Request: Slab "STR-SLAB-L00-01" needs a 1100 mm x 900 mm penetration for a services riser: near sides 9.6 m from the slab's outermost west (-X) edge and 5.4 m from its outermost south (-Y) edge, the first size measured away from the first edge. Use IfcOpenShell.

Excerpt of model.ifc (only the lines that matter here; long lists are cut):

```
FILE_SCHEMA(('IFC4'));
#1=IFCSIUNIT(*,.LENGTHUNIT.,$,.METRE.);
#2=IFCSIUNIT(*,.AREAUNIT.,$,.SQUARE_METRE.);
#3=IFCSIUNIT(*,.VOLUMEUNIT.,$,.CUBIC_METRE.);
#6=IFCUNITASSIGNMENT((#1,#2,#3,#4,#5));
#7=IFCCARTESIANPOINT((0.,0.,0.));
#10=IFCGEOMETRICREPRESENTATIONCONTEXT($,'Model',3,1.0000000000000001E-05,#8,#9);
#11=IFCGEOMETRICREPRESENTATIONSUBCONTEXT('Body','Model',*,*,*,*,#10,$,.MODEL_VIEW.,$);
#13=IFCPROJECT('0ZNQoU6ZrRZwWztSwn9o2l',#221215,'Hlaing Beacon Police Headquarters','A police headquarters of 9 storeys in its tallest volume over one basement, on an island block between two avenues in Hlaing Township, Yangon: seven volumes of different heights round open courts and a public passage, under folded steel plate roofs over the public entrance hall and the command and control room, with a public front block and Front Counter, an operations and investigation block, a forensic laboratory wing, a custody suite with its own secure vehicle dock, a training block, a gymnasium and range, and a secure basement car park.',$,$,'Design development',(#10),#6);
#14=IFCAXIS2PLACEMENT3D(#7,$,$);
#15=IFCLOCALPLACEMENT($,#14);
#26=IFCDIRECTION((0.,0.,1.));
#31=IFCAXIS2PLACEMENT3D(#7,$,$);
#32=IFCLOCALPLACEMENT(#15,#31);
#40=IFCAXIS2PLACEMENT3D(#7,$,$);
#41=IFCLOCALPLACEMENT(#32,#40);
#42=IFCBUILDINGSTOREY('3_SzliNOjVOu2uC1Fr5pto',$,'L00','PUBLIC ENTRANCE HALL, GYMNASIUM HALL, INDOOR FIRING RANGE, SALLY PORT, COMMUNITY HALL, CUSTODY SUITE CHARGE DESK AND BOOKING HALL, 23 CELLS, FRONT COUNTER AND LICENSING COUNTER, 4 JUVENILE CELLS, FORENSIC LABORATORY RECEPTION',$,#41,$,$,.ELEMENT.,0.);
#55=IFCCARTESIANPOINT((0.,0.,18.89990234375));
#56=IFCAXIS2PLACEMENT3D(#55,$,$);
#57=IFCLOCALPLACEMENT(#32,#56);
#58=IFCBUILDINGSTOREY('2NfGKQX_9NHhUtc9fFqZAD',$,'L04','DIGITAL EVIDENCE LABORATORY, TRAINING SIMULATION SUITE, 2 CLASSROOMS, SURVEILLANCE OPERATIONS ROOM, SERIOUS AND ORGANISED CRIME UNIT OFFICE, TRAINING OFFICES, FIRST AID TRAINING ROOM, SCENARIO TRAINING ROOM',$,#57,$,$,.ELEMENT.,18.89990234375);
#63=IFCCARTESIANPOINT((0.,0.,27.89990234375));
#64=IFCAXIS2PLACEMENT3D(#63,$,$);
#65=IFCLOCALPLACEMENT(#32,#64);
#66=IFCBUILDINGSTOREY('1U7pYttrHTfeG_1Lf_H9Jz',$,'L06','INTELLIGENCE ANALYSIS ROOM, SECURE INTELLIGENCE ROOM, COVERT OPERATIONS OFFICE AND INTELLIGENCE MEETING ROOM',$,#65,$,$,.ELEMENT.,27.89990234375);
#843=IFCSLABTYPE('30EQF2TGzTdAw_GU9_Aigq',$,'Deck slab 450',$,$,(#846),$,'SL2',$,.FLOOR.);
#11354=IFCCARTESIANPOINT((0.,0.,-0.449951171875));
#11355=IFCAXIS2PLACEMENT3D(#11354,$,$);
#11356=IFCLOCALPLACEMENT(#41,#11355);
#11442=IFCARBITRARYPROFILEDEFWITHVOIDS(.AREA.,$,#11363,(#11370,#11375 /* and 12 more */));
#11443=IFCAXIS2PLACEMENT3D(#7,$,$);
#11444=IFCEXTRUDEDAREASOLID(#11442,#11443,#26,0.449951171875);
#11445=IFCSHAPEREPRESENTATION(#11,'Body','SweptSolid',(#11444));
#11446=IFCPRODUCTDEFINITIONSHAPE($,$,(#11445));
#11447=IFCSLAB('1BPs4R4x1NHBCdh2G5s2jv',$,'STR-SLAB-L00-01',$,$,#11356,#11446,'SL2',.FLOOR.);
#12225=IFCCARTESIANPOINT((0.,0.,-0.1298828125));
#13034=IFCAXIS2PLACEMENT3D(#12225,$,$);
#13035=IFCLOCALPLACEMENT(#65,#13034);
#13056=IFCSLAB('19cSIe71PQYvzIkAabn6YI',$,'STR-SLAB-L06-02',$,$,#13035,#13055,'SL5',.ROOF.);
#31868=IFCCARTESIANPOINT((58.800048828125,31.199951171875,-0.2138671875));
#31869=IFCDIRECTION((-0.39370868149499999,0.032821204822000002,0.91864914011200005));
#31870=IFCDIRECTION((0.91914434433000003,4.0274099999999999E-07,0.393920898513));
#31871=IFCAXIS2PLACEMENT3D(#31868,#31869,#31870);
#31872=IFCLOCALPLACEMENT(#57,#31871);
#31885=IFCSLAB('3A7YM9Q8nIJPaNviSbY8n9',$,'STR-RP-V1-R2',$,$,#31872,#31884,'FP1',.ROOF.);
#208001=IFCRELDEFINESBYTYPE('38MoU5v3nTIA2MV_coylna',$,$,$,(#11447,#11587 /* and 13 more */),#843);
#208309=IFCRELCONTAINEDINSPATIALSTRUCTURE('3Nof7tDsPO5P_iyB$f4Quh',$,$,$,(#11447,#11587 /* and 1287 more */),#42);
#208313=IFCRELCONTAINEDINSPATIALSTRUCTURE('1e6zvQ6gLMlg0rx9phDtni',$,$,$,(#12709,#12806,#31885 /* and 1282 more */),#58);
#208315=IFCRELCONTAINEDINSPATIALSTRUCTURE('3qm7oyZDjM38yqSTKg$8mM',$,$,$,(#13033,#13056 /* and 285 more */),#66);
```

```python
import numpy as np
import ifcopenshell
import ifcopenshell.api.feature
import ifcopenshell.api.geometry
import ifcopenshell.api.root
import ifcopenshell.geom
import ifcopenshell.util.placement
import ifcopenshell.util.representation
import ifcopenshell.util.shape
import ifcopenshell.util.unit

model = ifcopenshell.open("model.ifc")
unit_scale = ifcopenshell.util.unit.calculate_unit_scale(model)
settings = ifcopenshell.geom.settings()


def volume(element):
    """Net volume in cubic metres, openings subtracted."""
    shape = ifcopenshell.geom.create_shape(settings, element)
    return ifcopenshell.util.shape.get_volume(shape.geometry)


slab = model.by_guid("1BPs4R4x1NHBCdh2G5s2jv")
before = volume(slab)

# Extent in the slab's own axes, in metres. The edges named are its -X and -Y sides.
slab_shape = ifcopenshell.geom.create_shape(settings, slab)
vertices = ifcopenshell.util.shape.get_vertices(slab_shape.geometry)
x_min, y_min, bottom = vertices.min(axis=0)
top = vertices[:, 2].max()

opening = ifcopenshell.api.root.create_entity(model, ifc_class="IfcOpeningElement", name="Services riser opening", predefined_type="OPENING")
context = ifcopenshell.util.representation.get_context(model, "Model", "Body", "MODEL_VIEW")
width, depth = 1.1, 0.9
outline = [(0.0, 0.0), (width, 0.0), (width, depth), (0.0, depth), (0.0, 0.0)]
# Overshoot both faces by 50 mm so the cut is clean.
shape = ifcopenshell.api.geometry.add_slab_representation(
    model, context=context, depth=top - bottom + 0.1, polyline=outline
)
ifcopenshell.api.geometry.assign_representation(model, product=opening, representation=shape)

matrix = ifcopenshell.util.placement.get_local_placement(slab.ObjectPlacement)
matrix[:, 3] = matrix @ np.append(np.array([x_min + 9.6, y_min + 5.4, bottom - 0.05]) / unit_scale, 1.0)
ifcopenshell.api.geometry.edit_object_placement(model, product=opening, matrix=matrix, is_si=False)
ifcopenshell.api.feature.add_feature(model, feature=opening, element=slab)

after = volume(slab)

print(f"slab volume {before:.3f} -> {after:.3f} m3")

model.write("model_updated.ifc")
```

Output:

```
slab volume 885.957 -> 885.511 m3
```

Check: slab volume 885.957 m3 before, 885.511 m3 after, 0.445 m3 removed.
